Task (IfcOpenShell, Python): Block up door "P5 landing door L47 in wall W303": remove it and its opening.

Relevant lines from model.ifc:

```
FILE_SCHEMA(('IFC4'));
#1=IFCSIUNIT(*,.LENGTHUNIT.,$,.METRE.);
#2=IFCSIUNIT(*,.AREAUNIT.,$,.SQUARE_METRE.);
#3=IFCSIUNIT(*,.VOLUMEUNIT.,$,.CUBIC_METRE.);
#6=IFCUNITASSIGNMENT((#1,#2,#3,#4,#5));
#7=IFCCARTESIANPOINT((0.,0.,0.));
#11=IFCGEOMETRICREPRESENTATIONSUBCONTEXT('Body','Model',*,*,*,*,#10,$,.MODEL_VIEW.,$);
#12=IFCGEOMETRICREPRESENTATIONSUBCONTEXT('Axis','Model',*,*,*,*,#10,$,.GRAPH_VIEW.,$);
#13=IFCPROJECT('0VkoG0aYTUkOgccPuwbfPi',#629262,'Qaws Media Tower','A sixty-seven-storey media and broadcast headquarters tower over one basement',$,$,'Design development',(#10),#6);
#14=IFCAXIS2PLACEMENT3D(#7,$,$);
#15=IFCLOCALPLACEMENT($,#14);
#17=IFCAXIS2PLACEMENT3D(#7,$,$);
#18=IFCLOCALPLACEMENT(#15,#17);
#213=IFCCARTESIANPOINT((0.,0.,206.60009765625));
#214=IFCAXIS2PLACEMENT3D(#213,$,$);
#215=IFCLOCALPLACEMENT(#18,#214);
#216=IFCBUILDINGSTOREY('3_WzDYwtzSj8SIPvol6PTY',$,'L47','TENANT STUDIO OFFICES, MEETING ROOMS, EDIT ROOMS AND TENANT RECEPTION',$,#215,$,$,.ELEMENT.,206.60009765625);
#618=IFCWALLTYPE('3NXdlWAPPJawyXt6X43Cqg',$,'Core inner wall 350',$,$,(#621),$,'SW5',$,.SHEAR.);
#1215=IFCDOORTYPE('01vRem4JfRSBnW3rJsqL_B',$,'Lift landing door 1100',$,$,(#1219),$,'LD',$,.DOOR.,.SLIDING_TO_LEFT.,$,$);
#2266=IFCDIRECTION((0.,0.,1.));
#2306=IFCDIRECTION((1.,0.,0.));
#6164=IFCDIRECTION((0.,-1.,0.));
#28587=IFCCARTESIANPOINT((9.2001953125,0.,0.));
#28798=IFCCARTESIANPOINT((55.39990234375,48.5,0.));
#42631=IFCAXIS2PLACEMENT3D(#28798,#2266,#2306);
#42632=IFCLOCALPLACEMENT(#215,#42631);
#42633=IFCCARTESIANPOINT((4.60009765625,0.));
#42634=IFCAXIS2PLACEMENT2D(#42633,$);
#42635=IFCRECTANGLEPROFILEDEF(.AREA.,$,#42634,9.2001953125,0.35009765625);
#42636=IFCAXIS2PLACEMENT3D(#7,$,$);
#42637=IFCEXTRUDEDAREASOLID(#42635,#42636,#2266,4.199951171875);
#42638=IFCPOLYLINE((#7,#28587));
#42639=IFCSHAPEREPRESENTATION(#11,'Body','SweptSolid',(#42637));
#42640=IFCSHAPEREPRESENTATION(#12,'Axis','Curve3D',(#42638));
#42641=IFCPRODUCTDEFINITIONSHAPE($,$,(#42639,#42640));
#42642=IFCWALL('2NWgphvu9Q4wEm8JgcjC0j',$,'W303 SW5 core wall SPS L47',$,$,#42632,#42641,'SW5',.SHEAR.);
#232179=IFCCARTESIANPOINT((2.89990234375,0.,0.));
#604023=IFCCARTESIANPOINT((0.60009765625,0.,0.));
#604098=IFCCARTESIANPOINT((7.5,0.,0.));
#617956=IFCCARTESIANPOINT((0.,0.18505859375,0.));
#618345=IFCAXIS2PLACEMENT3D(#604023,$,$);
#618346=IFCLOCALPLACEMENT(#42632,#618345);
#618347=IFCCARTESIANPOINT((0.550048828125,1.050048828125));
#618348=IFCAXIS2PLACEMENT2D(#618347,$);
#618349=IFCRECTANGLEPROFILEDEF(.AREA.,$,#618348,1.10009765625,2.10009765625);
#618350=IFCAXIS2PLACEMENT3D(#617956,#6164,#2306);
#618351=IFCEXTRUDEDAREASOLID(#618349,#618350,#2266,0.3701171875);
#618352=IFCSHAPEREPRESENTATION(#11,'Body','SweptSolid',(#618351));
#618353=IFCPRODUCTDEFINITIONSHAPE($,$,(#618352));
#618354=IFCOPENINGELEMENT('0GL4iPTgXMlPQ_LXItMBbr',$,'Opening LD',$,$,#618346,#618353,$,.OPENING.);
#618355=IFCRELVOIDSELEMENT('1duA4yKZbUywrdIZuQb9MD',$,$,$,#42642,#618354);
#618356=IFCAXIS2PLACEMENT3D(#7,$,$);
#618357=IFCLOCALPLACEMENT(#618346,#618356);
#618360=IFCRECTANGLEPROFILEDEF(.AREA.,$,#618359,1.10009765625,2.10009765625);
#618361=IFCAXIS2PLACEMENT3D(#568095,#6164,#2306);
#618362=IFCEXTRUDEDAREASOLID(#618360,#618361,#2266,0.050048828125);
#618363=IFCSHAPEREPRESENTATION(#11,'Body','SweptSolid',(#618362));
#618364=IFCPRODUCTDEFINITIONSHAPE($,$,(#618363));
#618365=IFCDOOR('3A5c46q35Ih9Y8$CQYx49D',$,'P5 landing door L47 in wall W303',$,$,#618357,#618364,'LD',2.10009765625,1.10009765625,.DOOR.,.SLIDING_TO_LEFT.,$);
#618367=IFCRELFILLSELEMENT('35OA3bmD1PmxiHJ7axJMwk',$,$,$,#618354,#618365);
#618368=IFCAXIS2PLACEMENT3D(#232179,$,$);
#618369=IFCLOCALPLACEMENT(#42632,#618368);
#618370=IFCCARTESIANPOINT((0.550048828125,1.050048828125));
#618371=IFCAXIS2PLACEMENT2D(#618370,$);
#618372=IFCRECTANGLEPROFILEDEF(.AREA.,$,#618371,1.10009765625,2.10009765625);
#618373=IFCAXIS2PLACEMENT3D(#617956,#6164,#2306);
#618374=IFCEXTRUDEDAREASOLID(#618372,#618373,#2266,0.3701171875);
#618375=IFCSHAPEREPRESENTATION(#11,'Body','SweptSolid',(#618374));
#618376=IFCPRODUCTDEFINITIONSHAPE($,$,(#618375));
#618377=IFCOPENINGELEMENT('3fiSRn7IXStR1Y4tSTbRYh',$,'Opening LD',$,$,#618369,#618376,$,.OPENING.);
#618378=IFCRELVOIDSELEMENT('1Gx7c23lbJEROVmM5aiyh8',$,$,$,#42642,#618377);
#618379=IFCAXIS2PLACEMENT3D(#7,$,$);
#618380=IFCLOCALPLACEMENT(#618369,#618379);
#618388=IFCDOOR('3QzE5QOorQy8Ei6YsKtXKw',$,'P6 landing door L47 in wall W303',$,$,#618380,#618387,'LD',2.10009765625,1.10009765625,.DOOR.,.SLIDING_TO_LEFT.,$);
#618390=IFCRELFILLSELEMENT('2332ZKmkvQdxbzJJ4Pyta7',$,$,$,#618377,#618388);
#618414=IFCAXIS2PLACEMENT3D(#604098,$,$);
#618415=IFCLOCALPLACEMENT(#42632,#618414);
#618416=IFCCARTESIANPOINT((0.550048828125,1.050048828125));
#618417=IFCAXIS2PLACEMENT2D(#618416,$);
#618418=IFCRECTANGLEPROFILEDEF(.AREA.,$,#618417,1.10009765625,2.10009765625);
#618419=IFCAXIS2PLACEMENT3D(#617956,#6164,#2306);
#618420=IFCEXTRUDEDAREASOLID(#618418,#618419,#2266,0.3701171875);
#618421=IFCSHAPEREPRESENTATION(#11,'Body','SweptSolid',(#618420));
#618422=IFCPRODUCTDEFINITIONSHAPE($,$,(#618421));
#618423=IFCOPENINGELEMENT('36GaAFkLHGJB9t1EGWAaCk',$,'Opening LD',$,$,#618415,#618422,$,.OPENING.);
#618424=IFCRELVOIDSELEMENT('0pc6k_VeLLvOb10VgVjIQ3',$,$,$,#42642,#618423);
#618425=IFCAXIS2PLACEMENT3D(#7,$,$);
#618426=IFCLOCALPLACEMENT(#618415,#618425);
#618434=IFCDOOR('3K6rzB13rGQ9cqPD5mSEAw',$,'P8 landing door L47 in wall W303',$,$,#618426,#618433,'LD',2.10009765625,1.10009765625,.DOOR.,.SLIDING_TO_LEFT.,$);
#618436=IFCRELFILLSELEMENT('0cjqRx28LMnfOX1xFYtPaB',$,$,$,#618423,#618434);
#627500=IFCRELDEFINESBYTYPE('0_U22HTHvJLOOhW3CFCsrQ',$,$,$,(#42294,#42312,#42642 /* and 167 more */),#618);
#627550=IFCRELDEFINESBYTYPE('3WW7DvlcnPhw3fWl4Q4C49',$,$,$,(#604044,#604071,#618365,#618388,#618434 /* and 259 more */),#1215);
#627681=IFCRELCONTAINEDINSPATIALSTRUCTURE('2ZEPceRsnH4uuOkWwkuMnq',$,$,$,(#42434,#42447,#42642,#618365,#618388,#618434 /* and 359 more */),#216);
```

```python
import ifcopenshell
import ifcopenshell.api.feature
import ifcopenshell.api.root
import ifcopenshell.geom
import ifcopenshell.util.shape

model = ifcopenshell.open("model.ifc")
settings = ifcopenshell.geom.settings()


def volume(element):
    """Net volume in cubic metres, openings subtracted."""
    shape = ifcopenshell.geom.create_shape(settings, element)
    return ifcopenshell.util.shape.get_volume(shape.geometry)


door = model.by_guid("3A5c46q35Ih9Y8$CQYx49D")
opening = door.FillsVoids[0].RelatingOpeningElement
wall = opening.VoidsElements[0].RelatingBuildingElement
before = volume(wall)

ifcopenshell.api.root.remove_product(model, product=door)
ifcopenshell.api.feature.remove_feature(model, feature=opening)

after = volume(wall)

print(f"wall volume {before:.3f} -> {after:.3f} m3")

model.write("model_edited.ifc")
```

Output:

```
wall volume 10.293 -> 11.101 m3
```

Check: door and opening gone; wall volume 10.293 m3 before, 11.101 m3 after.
